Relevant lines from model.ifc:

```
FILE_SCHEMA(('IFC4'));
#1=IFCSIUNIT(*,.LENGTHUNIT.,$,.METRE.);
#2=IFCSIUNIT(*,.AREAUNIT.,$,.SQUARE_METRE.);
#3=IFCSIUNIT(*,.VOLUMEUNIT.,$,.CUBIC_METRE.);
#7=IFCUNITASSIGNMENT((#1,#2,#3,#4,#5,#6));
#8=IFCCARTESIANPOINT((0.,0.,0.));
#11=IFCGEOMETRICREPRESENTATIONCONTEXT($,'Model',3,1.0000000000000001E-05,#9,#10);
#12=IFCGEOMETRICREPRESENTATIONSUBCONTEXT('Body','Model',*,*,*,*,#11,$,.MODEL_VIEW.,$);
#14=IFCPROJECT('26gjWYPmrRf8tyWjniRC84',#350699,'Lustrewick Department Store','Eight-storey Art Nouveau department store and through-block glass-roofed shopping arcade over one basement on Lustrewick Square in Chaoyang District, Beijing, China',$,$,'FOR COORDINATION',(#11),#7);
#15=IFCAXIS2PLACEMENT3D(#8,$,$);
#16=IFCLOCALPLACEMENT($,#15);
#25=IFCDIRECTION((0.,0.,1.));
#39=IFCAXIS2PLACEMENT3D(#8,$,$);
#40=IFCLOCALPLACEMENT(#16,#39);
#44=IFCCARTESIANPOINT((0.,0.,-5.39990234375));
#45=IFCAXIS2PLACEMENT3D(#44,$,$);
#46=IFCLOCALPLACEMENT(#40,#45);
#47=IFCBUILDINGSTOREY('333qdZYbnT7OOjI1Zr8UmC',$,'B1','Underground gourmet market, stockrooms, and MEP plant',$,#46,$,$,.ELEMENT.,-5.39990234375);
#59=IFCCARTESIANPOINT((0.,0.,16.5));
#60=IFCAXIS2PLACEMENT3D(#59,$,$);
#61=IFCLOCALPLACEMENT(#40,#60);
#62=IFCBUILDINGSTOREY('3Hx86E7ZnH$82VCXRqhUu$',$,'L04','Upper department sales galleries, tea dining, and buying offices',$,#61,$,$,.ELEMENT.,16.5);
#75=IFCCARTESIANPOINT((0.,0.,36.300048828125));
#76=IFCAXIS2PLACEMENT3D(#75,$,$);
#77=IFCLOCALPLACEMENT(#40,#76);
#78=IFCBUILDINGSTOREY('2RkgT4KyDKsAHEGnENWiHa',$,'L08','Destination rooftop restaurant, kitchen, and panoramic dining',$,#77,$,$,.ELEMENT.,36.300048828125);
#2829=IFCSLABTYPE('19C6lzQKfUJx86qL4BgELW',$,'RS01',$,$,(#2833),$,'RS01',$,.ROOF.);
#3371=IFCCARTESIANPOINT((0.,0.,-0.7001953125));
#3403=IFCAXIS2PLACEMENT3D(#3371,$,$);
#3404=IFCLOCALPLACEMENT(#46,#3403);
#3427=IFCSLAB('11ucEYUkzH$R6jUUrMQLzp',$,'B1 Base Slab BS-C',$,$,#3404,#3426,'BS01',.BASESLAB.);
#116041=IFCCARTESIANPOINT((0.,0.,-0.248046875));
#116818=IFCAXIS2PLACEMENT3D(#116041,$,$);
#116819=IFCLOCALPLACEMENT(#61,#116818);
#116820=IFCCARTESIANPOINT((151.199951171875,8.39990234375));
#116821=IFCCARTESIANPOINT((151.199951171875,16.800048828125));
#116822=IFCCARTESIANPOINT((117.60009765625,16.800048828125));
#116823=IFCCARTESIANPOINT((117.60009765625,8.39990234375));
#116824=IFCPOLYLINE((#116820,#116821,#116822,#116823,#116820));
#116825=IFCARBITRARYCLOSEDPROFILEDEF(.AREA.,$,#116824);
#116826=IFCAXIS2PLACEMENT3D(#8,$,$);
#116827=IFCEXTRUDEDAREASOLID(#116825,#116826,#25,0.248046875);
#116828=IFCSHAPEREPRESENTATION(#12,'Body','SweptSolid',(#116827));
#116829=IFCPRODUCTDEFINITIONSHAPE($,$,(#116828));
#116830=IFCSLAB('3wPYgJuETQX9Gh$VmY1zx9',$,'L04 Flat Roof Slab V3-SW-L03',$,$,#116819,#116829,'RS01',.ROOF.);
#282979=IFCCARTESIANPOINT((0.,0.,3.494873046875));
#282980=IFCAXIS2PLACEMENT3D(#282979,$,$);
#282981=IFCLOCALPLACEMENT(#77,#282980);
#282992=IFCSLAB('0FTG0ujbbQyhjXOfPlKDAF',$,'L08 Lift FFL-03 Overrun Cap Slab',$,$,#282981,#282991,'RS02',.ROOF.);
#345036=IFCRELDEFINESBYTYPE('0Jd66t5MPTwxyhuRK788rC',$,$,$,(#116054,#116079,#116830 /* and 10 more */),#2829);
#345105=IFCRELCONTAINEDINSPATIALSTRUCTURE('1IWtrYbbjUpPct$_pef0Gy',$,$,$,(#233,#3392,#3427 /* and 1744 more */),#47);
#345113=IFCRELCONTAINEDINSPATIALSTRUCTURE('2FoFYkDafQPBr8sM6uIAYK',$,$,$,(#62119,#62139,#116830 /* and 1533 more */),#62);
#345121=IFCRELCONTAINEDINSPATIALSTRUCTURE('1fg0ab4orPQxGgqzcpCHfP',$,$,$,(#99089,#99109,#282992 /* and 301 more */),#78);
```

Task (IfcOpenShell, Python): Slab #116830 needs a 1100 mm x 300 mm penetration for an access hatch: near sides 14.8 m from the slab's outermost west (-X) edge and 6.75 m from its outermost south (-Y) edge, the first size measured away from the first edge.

```python
import numpy as np
import ifcopenshell
import ifcopenshell.api.feature
import ifcopenshell.api.geometry
import ifcopenshell.api.root
import ifcopenshell.geom
import ifcopenshell.util.placement
import ifcopenshell.util.representation
import ifcopenshell.util.shape
import ifcopenshell.util.unit

model = ifcopenshell.open("model.ifc")
unit_scale = ifcopenshell.util.unit.calculate_unit_scale(model)
settings = ifcopenshell.geom.settings()


def volume(element):
    """Net volume in cubic metres, openings subtracted."""
    shape = ifcopenshell.geom.create_shape(settings, element)
    return ifcopenshell.util.shape.get_volume(shape.geometry)


slab = model.by_guid("3wPYgJuETQX9Gh$VmY1zx9")
before = volume(slab)

# Extent in the slab's own axes, in metres. The edges named are its -X and -Y sides.
slab_shape = ifcopenshell.geom.create_shape(settings, slab)
vertices = ifcopenshell.util.shape.get_vertices(slab_shape.geometry)
x_min, y_min, bottom = vertices.min(axis=0)
top = vertices[:, 2].max()

opening = ifcopenshell.api.root.create_entity(model, ifc_class="IfcOpeningElement", name="Access hatch opening", predefined_type="OPENING")
context = ifcopenshell.util.representation.get_context(model, "Model", "Body", "MODEL_VIEW")
width, depth = 1.1, 0.3
outline = [(0.0, 0.0), (width, 0.0), (width, depth), (0.0, depth), (0.0, 0.0)]
# Overshoot both faces by 50 mm so the cut is clean.
shape = ifcopenshell.api.geometry.add_slab_representation(
    model, context=context, depth=top - bottom + 0.1, polyline=outline
)
ifcopenshell.api.geometry.assign_representation(model, product=opening, representation=shape)

matrix = ifcopenshell.util.placement.get_local_placement(slab.ObjectPlacement)
matrix[:, 3] = matrix @ np.append(np.array([x_min + 14.8, y_min + 6.75, bottom - 0.05]) / unit_scale, 1.0)
ifcopenshell.api.geometry.edit_object_placement(model, product=opening, matrix=matrix, is_si=False)
ifcopenshell.api.feature.add_feature(model, feature=opening, element=slab)

after = volume(slab)

print(f"slab volume {before:.3f} -> {after:.3f} m3")

model.write("model_v2.ifc")
```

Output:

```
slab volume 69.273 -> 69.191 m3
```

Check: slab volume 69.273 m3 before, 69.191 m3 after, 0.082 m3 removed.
